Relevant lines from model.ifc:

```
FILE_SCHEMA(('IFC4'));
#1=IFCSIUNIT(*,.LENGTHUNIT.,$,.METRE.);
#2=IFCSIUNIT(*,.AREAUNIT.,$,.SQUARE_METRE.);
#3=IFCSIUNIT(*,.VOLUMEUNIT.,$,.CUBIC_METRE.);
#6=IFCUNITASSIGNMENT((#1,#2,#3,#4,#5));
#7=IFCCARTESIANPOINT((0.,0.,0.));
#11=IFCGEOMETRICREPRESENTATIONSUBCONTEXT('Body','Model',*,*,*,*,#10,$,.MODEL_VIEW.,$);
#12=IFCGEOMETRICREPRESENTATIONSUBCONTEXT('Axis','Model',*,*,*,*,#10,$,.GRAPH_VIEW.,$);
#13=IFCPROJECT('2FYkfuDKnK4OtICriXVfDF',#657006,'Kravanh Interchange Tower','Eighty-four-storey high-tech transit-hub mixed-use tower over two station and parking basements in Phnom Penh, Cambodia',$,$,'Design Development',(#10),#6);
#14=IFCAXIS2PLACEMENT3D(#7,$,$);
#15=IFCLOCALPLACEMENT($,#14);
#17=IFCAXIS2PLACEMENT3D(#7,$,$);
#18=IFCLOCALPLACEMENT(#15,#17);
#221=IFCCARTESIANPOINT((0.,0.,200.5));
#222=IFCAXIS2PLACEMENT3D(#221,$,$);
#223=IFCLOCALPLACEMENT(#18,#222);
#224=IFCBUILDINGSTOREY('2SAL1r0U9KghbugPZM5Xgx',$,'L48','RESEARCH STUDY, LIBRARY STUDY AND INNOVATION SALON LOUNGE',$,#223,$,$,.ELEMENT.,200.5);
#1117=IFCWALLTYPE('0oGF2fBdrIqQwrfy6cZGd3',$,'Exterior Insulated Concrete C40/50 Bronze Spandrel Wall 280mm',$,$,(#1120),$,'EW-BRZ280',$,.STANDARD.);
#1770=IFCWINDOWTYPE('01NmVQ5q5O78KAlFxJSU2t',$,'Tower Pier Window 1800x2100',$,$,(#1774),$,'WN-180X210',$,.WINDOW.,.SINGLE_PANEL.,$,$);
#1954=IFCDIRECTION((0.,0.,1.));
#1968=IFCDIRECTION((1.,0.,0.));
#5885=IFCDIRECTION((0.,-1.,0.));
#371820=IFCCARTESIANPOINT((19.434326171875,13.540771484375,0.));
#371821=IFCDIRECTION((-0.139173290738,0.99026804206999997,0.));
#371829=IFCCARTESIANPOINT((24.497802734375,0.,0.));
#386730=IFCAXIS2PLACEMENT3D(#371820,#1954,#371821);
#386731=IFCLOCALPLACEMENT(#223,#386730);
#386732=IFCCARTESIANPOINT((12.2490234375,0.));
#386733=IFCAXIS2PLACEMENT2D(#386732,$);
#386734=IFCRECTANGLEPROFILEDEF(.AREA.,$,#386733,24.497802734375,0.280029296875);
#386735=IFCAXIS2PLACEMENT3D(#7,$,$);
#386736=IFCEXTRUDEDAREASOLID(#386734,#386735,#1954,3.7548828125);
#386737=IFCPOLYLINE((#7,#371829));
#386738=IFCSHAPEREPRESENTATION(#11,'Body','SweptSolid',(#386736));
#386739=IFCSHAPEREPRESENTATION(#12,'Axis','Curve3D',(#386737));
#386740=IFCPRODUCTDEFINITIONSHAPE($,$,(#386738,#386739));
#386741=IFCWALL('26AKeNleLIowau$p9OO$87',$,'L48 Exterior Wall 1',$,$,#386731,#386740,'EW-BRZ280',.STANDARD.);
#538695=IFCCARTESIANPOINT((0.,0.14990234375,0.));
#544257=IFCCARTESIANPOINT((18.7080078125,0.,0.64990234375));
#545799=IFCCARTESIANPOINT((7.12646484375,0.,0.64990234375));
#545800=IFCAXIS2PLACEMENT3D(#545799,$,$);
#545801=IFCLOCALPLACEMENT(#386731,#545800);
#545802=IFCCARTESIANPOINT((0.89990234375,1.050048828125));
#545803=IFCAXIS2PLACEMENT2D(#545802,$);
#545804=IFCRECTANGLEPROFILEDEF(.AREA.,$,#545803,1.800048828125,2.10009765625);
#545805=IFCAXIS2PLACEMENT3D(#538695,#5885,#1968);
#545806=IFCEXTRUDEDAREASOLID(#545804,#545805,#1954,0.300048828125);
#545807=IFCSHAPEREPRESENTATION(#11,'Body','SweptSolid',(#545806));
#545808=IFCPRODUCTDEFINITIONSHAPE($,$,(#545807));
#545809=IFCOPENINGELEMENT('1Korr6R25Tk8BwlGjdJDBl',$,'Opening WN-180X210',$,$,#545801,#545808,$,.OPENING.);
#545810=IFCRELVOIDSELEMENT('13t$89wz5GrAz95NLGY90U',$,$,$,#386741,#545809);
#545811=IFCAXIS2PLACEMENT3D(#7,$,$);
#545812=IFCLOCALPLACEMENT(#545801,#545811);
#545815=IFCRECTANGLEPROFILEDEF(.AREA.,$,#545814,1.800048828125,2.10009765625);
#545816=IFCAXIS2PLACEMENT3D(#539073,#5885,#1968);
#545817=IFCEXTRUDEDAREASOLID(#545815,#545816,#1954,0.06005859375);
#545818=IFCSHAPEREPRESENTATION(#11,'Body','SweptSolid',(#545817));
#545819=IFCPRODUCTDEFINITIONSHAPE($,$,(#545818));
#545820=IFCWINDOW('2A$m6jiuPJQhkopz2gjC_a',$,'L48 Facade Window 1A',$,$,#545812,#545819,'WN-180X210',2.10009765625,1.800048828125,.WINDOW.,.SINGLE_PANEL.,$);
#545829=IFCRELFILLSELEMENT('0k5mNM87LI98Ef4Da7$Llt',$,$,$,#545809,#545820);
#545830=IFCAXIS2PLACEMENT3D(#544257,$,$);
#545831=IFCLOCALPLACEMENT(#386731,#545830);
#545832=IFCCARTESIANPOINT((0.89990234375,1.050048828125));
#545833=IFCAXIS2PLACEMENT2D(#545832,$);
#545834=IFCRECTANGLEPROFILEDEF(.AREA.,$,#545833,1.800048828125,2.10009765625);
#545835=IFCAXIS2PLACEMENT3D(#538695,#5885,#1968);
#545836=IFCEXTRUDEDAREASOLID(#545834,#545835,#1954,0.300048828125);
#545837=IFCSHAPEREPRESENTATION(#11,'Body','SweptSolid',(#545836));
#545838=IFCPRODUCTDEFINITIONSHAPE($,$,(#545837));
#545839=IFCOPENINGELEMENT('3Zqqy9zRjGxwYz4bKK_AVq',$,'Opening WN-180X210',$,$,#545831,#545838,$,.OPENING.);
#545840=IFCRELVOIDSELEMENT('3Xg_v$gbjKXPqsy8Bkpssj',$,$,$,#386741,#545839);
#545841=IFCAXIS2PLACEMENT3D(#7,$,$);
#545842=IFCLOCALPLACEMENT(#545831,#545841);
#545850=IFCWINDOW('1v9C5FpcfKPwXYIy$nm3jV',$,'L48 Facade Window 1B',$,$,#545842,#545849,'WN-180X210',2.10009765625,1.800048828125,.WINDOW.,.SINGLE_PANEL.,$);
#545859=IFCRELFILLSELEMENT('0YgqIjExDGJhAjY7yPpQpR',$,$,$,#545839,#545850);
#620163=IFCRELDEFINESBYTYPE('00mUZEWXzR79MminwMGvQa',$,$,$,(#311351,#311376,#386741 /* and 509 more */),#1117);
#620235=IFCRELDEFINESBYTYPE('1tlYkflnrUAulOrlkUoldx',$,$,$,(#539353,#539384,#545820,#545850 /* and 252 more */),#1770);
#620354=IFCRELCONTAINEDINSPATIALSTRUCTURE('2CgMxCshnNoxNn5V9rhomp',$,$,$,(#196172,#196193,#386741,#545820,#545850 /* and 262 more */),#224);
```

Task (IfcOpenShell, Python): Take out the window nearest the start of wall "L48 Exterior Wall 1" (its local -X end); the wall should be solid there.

```python
import ifcopenshell
import ifcopenshell.api.feature
import ifcopenshell.api.root
import ifcopenshell.geom
import ifcopenshell.util.shape

model = ifcopenshell.open("model.ifc")
settings = ifcopenshell.geom.settings()


def volume(element):
    """Net volume in cubic metres, openings subtracted."""
    shape = ifcopenshell.geom.create_shape(settings, element)
    return ifcopenshell.util.shape.get_volume(shape.geometry)


window = model.by_guid("2A$m6jiuPJQhkopz2gjC_a")
opening = window.FillsVoids[0].RelatingOpeningElement
wall = opening.VoidsElements[0].RelatingBuildingElement
before = volume(wall)

ifcopenshell.api.root.remove_product(model, product=window)
ifcopenshell.api.feature.remove_feature(model, feature=opening)

after = volume(wall)

print(f"wall volume {before:.3f} -> {after:.3f} m3")

model.write("model_rev.ifc")
```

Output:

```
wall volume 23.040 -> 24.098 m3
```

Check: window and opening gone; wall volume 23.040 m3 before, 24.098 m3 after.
